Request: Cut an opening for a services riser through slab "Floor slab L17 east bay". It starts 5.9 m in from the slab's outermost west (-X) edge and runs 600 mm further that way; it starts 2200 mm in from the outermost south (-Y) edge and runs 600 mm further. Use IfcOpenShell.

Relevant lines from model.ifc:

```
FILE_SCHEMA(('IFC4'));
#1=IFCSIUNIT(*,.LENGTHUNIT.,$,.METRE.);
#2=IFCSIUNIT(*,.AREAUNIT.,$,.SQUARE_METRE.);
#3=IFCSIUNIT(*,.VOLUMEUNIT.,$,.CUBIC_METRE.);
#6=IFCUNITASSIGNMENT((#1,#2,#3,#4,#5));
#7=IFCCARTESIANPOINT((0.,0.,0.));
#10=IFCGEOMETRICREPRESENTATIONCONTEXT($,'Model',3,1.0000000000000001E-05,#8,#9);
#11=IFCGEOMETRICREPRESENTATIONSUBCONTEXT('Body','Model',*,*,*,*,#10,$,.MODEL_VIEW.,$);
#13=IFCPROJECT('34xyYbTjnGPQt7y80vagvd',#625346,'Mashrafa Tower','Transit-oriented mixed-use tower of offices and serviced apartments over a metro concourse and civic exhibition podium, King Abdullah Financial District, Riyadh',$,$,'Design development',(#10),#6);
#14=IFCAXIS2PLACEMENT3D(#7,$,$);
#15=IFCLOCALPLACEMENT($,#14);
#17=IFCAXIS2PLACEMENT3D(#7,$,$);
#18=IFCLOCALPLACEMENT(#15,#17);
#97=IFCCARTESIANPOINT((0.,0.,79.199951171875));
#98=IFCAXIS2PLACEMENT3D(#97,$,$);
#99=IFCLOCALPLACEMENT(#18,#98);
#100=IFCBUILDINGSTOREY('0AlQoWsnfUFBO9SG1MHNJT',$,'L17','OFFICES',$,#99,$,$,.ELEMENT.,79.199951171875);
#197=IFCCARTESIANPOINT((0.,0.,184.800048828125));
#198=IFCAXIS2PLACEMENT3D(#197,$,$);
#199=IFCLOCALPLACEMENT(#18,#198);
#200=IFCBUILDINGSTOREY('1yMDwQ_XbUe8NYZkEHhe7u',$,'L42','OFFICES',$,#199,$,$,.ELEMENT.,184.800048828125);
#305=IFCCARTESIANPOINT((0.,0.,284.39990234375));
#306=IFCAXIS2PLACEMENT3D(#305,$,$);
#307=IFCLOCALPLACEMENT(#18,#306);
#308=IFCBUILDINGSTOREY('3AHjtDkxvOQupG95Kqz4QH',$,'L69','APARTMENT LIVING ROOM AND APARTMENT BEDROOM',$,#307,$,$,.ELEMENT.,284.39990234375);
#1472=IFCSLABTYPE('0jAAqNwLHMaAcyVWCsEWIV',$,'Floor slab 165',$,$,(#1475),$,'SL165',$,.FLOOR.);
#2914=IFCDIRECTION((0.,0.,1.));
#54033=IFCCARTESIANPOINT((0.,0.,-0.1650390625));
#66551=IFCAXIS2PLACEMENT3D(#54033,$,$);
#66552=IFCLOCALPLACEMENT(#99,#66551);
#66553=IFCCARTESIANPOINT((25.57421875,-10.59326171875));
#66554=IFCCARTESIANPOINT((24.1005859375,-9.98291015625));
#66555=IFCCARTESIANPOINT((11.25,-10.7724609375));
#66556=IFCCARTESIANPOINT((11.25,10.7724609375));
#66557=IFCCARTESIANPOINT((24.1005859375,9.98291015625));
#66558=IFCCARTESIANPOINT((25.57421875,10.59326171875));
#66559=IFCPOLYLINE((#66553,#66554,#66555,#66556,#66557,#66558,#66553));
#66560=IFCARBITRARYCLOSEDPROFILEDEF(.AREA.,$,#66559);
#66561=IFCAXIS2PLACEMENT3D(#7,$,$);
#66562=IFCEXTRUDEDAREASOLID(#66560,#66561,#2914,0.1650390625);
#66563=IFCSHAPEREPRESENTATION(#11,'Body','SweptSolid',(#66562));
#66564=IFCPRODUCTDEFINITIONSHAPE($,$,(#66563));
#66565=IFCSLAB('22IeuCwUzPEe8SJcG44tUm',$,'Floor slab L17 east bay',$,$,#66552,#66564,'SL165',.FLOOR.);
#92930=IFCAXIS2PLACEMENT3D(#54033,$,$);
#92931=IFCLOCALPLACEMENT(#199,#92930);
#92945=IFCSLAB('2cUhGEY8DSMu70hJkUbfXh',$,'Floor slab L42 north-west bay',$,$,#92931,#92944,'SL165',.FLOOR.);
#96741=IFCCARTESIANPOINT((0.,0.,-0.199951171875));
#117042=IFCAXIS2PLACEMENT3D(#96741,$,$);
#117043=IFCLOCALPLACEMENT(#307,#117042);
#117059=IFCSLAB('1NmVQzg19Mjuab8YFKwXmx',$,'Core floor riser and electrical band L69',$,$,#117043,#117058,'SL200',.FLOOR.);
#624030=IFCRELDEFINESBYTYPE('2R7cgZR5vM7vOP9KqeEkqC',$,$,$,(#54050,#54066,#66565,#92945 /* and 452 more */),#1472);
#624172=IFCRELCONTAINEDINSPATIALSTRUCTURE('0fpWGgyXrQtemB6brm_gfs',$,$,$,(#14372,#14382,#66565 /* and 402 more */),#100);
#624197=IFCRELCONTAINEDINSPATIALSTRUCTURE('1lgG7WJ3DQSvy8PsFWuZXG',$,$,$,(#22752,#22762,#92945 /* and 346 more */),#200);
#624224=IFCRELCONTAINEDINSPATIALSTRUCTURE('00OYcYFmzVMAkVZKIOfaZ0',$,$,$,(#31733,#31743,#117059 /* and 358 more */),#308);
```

```python
import numpy as np
import ifcopenshell
import ifcopenshell.api.feature
import ifcopenshell.api.geometry
import ifcopenshell.api.root
import ifcopenshell.geom
import ifcopenshell.util.placement
import ifcopenshell.util.representation
import ifcopenshell.util.shape
import ifcopenshell.util.unit

model = ifcopenshell.open("model.ifc")
unit_scale = ifcopenshell.util.unit.calculate_unit_scale(model)
settings = ifcopenshell.geom.settings()


def volume(element):
    """Net volume in cubic metres, openings subtracted."""
    shape = ifcopenshell.geom.create_shape(settings, element)
    return ifcopenshell.util.shape.get_volume(shape.geometry)


slab = model.by_guid("22IeuCwUzPEe8SJcG44tUm")
before = volume(slab)

# Extent in the slab's own axes, in metres. The edges named are its -X and -Y sides.
slab_shape = ifcopenshell.geom.create_shape(settings, slab)
vertices = ifcopenshell.util.shape.get_vertices(slab_shape.geometry)
x_min, y_min, bottom = vertices.min(axis=0)
top = vertices[:, 2].max()

opening = ifcopenshell.api.root.create_entity(model, ifc_class="IfcOpeningElement", name="Services riser opening", predefined_type="OPENING")
context = ifcopenshell.util.representation.get_context(model, "Model", "Body", "MODEL_VIEW")
width, depth = 0.6, 0.6
outline = [(0.0, 0.0), (width, 0.0), (width, depth), (0.0, depth), (0.0, 0.0)]
# Overshoot both faces by 50 mm so the cut is clean.
shape = ifcopenshell.api.geometry.add_slab_representation(
    model, context=context, depth=top - bottom + 0.1, polyline=outline
)
ifcopenshell.api.geometry.assign_representation(model, product=opening, representation=shape)

matrix = ifcopenshell.util.placement.get_local_placement(slab.ObjectPlacement)
matrix[:, 3] = matrix @ np.append(np.array([x_min + 5.9, y_min + 2.2, bottom - 0.05]) / unit_scale, 1.0)
ifcopenshell.api.geometry.edit_object_placement(model, product=opening, matrix=matrix, is_si=False)
ifcopenshell.api.feature.add_feature(model, feature=opening, element=slab)

after = volume(slab)

print(f"slab volume {before:.3f} -> {after:.3f} m3")

model.write("model_updated.ifc")
```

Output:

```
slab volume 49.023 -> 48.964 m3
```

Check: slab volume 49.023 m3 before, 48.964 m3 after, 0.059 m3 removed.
